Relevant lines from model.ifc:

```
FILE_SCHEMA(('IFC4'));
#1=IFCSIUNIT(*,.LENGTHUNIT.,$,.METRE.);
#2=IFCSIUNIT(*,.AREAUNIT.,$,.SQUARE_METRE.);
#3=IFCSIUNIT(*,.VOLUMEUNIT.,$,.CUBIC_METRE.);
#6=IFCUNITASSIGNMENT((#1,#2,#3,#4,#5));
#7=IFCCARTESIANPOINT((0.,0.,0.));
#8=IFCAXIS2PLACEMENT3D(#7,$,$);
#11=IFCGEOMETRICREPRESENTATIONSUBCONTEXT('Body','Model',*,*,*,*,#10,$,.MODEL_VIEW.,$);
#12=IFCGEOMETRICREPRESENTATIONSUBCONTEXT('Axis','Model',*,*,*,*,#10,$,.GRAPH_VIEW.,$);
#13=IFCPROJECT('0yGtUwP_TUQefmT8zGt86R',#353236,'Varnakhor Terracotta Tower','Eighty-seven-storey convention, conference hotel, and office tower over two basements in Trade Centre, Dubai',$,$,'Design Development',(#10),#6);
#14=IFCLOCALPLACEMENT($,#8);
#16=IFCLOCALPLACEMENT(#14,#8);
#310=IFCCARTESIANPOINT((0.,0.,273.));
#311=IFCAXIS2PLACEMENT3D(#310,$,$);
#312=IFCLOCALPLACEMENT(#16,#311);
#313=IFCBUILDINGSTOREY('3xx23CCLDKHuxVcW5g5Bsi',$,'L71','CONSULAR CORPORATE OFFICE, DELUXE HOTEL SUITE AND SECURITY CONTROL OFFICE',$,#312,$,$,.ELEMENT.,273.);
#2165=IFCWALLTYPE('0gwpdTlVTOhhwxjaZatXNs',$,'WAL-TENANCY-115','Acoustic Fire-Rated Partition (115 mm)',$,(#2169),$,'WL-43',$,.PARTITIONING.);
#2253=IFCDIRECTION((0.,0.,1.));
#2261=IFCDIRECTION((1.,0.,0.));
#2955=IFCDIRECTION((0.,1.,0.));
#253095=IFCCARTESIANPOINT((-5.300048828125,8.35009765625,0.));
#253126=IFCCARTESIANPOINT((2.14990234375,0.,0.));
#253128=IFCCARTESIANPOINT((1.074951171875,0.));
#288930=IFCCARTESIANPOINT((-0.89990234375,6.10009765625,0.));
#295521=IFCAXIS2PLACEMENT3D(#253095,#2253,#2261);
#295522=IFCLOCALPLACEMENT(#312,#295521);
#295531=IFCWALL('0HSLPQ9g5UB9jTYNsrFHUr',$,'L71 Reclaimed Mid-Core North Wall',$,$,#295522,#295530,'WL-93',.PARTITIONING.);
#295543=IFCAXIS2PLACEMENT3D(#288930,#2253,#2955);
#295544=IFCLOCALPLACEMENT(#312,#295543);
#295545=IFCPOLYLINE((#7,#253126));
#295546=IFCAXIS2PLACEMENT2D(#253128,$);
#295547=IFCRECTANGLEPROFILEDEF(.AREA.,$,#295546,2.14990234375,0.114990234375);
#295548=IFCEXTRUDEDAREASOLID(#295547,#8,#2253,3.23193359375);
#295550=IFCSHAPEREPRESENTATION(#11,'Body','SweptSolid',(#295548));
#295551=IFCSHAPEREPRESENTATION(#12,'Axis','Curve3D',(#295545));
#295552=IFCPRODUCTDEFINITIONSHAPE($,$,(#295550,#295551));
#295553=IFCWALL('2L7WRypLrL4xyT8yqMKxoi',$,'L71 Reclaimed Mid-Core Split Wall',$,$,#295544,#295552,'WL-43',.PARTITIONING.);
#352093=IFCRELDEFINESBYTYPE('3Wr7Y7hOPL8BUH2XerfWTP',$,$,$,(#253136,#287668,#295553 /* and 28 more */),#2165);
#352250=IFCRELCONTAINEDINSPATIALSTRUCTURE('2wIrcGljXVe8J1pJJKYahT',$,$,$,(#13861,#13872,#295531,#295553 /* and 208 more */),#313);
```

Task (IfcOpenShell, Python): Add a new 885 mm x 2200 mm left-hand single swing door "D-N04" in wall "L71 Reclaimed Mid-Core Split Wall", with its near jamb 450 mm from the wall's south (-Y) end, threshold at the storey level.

```python
import numpy as np
import ifcopenshell
import ifcopenshell.api.feature
import ifcopenshell.api.geometry
import ifcopenshell.api.root
import ifcopenshell.api.spatial
import ifcopenshell.geom
import ifcopenshell.util.element
import ifcopenshell.util.placement
import ifcopenshell.util.representation
import ifcopenshell.util.shape
import ifcopenshell.util.unit

model = ifcopenshell.open("model.ifc")
unit_scale = ifcopenshell.util.unit.calculate_unit_scale(model)
settings = ifcopenshell.geom.settings()


def volume(element):
    """Net volume in cubic metres, openings subtracted."""
    shape = ifcopenshell.geom.create_shape(settings, element)
    return ifcopenshell.util.shape.get_volume(shape.geometry)


wall = model.by_id(295553)
storey = ifcopenshell.util.element.get_container(wall, ifc_class="IfcBuildingStorey")
context = ifcopenshell.util.representation.get_context(model, "Model", "Body", "MODEL_VIEW")
before = volume(wall)

width, height, from_end, sill = 0.885, 2.2, 0.45, 0.0  # metres

# The wall runs along its own X axis, and the end named is its -X end.
wall_shape = ifcopenshell.geom.create_shape(settings, wall)
x, y, z = ifcopenshell.util.shape.get_vertices(wall_shape.geometry).T
start = x.min() + from_end
face, thickness = float(y.min()), float(y.max() - y.min())
wall_matrix = ifcopenshell.util.placement.get_local_placement(wall.ObjectPlacement)
level = ifcopenshell.util.placement.get_local_placement(storey.ObjectPlacement)[2, 3]


def in_wall(x, y):
    """Placement at x, y metres in the wall's axes, at sill height."""
    matrix = wall_matrix.copy()
    matrix[:, 3] = wall_matrix @ np.array([x / unit_scale, y / unit_scale, 0.0, 1.0])
    matrix[2, 3] = level + sill / unit_scale
    return matrix


# Opening: a box that overshoots both wall faces by 50 mm.
opening = ifcopenshell.api.root.create_entity(model, ifc_class="IfcOpeningElement", predefined_type="OPENING")
box = ifcopenshell.api.geometry.add_wall_representation(
    model, context=context, length=width, height=height, thickness=thickness + 0.1
)
ifcopenshell.api.geometry.assign_representation(model, product=opening, representation=box)
ifcopenshell.api.geometry.edit_object_placement(model, product=opening, matrix=in_wall(start, face - 0.05), is_si=False)
ifcopenshell.api.feature.add_feature(model, feature=opening, element=wall)

door = ifcopenshell.api.root.create_entity(model, ifc_class="IfcDoor", name="D-N04", predefined_type="DOOR")
door.OverallWidth, door.OverallHeight = width / unit_scale, height / unit_scale
door.OperationType = "SINGLE_SWING_LEFT"
body = ifcopenshell.api.geometry.add_door_representation(
    model,
    context=context,
    overall_width=door.OverallWidth,
    overall_height=door.OverallHeight,
    operation_type="SINGLE_SWING_LEFT",
    lining_properties={"LiningDepth": thickness / unit_scale, "ThresholdDepth": thickness / unit_scale},
)
ifcopenshell.api.geometry.assign_representation(model, product=door, representation=body)
ifcopenshell.api.spatial.assign_container(model, products=[door], relating_structure=storey)
ifcopenshell.api.feature.add_filling(model, opening=opening, element=door)

# The lining spans the wall, so the door starts at the wall face.
ifcopenshell.api.geometry.edit_object_placement(model, product=door, matrix=in_wall(start, face), is_si=False)

after = volume(wall)

print(f"wall volume {before:.3f} -> {after:.3f} m3")

model.write("model-out.ifc")
```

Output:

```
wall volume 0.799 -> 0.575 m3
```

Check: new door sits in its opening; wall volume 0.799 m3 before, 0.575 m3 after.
